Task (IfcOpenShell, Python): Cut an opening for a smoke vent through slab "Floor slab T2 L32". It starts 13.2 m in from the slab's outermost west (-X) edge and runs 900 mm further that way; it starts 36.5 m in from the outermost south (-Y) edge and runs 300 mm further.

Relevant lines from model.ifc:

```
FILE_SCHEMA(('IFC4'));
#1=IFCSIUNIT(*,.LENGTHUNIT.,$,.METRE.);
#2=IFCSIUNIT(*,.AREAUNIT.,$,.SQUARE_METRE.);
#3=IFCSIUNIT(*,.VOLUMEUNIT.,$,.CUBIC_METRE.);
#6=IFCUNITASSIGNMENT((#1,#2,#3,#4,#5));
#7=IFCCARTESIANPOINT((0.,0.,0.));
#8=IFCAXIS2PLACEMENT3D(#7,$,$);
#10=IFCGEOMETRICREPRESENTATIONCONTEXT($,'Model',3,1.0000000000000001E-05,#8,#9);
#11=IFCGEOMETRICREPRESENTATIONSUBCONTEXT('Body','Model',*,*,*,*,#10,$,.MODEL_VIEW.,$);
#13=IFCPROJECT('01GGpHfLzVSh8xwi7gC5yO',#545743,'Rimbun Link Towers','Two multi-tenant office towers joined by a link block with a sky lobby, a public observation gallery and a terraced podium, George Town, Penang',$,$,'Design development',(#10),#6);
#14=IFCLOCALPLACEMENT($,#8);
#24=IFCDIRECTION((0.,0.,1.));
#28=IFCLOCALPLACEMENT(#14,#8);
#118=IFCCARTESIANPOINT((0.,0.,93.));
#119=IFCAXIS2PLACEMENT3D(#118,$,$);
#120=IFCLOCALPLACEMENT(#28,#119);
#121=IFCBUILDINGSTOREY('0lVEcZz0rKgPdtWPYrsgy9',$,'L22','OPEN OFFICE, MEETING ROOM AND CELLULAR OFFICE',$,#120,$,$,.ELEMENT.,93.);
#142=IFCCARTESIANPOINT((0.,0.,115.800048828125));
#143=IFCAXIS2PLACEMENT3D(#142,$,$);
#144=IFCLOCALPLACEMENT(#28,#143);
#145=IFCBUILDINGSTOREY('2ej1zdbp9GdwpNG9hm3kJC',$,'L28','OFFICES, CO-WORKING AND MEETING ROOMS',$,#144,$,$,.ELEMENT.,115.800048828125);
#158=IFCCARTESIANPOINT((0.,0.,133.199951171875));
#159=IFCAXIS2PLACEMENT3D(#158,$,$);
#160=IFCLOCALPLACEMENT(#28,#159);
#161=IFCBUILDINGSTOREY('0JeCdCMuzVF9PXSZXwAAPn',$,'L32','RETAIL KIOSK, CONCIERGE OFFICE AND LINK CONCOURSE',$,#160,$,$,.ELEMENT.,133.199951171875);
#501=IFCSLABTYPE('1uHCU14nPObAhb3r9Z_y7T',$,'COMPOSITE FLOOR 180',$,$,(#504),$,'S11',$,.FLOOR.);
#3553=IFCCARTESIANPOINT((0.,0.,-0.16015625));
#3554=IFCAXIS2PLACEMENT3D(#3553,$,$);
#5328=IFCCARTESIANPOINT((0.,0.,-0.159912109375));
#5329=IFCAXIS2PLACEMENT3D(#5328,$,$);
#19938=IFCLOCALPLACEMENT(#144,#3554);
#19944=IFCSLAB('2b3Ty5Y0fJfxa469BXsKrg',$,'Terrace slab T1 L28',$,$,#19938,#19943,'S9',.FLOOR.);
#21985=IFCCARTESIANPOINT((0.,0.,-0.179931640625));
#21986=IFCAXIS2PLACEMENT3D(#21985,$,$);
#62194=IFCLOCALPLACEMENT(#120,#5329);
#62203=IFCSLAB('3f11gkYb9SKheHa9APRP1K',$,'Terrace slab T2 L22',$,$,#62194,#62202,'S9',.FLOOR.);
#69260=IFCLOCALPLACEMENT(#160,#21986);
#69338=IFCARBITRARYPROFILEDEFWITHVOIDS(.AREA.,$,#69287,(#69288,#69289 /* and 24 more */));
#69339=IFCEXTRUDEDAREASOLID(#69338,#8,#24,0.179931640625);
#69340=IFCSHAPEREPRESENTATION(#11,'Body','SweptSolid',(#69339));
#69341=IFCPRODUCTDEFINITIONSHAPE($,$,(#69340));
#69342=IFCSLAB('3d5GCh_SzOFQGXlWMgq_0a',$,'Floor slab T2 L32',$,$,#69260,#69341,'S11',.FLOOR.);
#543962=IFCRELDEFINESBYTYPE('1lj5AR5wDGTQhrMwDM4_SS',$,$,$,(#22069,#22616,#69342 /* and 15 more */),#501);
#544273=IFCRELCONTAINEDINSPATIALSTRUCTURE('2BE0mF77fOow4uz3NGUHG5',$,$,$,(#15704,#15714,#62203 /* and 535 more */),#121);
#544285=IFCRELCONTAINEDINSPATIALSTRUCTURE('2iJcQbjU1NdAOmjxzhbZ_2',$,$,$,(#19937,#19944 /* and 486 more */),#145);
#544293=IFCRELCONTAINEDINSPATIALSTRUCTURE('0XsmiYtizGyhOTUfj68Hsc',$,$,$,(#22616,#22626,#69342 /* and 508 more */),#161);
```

```python
import numpy as np
import ifcopenshell
import ifcopenshell.api.feature
import ifcopenshell.api.geometry
import ifcopenshell.api.root
import ifcopenshell.geom
import ifcopenshell.util.placement
import ifcopenshell.util.representation
import ifcopenshell.util.shape
import ifcopenshell.util.unit

model = ifcopenshell.open("model.ifc")
unit_scale = ifcopenshell.util.unit.calculate_unit_scale(model)
settings = ifcopenshell.geom.settings()


def volume(element):
    """Net volume in cubic metres, openings subtracted."""
    shape = ifcopenshell.geom.create_shape(settings, element)
    return ifcopenshell.util.shape.get_volume(shape.geometry)


slab = model.by_id(69342)
before = volume(slab)

# Extent in the slab's own axes, in metres. The edges named are its -X and -Y sides.
slab_shape = ifcopenshell.geom.create_shape(settings, slab)
vertices = ifcopenshell.util.shape.get_vertices(slab_shape.geometry)
x_min, y_min, bottom = vertices.min(axis=0)
top = vertices[:, 2].max()

opening = ifcopenshell.api.root.create_entity(model, ifc_class="IfcOpeningElement", name="Smoke vent opening", predefined_type="OPENING")
context = ifcopenshell.util.representation.get_context(model, "Model", "Body", "MODEL_VIEW")
width, depth = 0.9, 0.3
outline = [(0.0, 0.0), (width, 0.0), (width, depth), (0.0, depth), (0.0, 0.0)]
# Overshoot both faces by 50 mm so the cut is clean.
shape = ifcopenshell.api.geometry.add_slab_representation(
    model, context=context, depth=top - bottom + 0.1, polyline=outline
)
ifcopenshell.api.geometry.assign_representation(model, product=opening, representation=shape)

matrix = ifcopenshell.util.placement.get_local_placement(slab.ObjectPlacement)
matrix[:, 3] = matrix @ np.append(np.array([x_min + 13.2, y_min + 36.5, bottom - 0.05]) / unit_scale, 1.0)
ifcopenshell.api.geometry.edit_object_placement(model, product=opening, matrix=matrix, is_si=False)
ifcopenshell.api.feature.add_feature(model, feature=opening, element=slab)

after = volume(slab)

print(f"slab volume {before:.3f} -> {after:.3f} m3")

model.write("model_v2.ifc")
```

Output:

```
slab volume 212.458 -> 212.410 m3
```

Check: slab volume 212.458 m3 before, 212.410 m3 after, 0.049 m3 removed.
